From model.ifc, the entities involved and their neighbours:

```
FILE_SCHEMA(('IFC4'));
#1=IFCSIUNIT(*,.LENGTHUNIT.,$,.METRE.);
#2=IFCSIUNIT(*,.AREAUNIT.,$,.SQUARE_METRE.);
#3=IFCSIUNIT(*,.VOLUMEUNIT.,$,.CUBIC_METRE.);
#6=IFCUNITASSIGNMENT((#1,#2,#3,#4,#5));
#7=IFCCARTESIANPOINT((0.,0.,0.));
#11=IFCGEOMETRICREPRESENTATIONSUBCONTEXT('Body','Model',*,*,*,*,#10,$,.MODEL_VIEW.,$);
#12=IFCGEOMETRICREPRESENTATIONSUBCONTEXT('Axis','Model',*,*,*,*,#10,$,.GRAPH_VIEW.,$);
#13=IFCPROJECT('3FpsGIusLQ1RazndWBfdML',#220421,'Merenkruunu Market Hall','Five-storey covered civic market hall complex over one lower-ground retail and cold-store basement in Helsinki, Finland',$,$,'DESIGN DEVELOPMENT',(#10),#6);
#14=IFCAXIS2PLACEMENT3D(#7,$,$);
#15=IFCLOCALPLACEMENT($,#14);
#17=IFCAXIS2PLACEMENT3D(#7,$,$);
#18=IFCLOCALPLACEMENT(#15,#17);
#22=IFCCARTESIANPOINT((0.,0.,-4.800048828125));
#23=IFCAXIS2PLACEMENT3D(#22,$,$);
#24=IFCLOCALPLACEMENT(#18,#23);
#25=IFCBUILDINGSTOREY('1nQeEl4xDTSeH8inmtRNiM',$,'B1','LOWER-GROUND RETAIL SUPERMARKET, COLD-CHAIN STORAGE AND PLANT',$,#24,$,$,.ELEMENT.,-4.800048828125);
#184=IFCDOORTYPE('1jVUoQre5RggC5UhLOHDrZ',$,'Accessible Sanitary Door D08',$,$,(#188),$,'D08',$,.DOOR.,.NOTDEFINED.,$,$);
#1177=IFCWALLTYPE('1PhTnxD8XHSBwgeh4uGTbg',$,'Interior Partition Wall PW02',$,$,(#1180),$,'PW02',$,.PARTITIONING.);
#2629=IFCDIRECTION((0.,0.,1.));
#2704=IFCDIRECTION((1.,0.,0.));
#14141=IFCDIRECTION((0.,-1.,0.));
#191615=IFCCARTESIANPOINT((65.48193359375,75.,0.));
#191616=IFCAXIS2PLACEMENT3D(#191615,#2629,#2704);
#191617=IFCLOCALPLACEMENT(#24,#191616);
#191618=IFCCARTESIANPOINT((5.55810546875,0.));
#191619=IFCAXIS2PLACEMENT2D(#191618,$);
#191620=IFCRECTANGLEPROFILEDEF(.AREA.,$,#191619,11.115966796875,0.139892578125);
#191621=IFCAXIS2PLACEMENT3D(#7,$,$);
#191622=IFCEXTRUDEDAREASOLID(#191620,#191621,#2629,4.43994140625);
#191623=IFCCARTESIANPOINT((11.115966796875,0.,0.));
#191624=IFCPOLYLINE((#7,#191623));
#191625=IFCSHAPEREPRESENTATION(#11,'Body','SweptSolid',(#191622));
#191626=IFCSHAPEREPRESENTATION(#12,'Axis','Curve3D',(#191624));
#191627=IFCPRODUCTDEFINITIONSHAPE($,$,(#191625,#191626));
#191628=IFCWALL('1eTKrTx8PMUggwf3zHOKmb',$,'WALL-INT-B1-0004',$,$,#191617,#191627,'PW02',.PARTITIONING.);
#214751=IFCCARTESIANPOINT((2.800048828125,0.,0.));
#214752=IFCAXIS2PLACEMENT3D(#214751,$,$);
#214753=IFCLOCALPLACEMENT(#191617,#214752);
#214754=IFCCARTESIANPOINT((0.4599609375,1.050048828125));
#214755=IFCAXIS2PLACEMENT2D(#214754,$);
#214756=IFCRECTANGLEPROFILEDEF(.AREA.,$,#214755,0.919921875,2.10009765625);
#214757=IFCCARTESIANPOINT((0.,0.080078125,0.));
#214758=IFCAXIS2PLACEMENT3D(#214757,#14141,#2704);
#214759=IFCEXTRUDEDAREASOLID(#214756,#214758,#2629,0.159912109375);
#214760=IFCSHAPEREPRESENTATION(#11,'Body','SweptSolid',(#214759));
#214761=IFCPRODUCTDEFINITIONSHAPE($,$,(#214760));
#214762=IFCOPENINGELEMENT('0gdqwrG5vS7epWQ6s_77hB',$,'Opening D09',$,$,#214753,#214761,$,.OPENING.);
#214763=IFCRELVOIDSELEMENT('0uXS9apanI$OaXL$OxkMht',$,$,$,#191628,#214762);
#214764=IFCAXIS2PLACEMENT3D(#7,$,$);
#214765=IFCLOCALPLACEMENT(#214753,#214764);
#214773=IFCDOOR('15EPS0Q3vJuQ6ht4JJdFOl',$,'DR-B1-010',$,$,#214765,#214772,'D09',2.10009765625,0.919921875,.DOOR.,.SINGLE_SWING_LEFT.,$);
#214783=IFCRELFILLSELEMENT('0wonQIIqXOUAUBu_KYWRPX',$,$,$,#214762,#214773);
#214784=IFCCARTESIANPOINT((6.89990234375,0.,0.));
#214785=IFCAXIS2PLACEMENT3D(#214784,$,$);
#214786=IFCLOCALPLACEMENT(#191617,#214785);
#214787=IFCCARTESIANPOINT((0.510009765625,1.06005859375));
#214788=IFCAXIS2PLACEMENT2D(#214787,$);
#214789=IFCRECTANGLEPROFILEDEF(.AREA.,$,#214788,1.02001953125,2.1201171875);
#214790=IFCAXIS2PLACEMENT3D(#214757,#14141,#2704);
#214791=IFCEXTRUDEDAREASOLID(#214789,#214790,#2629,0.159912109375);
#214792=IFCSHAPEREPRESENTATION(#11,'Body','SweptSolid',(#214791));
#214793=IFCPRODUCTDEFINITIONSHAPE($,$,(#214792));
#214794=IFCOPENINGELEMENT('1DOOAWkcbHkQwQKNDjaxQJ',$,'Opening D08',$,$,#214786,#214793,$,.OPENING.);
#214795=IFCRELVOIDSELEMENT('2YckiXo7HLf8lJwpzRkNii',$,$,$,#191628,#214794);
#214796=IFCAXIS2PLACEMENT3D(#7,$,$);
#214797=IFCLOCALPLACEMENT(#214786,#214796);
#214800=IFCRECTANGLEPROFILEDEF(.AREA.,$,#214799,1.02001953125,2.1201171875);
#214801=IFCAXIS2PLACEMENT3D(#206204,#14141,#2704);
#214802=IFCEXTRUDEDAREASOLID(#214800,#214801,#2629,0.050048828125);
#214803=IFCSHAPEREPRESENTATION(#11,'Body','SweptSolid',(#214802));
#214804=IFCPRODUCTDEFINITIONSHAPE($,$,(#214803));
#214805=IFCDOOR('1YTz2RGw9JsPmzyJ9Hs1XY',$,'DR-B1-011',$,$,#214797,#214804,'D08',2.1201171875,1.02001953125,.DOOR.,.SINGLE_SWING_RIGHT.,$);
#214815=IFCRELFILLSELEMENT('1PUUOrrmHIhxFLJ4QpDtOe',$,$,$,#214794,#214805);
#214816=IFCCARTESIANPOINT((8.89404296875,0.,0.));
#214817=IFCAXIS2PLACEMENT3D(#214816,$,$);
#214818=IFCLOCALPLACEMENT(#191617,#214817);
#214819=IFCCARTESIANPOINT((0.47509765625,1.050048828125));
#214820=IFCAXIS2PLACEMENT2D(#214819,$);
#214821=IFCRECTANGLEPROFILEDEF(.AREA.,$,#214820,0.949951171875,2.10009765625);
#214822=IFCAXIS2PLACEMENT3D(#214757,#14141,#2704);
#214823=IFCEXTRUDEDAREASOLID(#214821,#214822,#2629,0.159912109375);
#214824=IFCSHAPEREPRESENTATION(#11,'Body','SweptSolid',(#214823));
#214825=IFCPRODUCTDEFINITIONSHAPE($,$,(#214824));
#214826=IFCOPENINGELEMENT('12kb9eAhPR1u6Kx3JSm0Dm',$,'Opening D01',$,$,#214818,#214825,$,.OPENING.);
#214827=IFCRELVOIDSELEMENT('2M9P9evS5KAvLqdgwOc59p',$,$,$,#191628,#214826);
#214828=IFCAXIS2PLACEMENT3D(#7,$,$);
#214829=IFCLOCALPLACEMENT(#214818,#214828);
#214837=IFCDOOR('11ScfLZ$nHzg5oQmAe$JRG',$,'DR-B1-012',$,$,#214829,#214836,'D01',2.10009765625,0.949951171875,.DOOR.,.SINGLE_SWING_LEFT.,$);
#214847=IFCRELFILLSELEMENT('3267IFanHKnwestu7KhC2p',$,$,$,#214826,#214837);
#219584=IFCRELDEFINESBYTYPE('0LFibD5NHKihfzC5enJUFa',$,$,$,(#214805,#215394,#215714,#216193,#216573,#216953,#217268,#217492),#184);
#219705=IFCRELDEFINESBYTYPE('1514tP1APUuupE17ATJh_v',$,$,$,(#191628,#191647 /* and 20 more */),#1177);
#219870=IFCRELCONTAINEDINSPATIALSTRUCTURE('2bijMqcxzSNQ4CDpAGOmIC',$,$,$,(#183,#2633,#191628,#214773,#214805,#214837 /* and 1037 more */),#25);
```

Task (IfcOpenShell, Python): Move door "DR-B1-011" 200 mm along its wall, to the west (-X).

```python
import ifcopenshell
import ifcopenshell.api.geometry
import ifcopenshell.util.placement
import ifcopenshell.util.unit

model = ifcopenshell.open("model.ifc")
unit_scale = ifcopenshell.util.unit.calculate_unit_scale(model)

door = model.by_guid("1YTz2RGw9JsPmzyJ9Hs1XY")
opening = door.FillsVoids[0].RelatingOpeningElement
wall = opening.VoidsElements[0].RelatingBuildingElement

wall_matrix = ifcopenshell.util.placement.get_local_placement(wall.ObjectPlacement)
shift = wall_matrix[:3, 0] * -0.2 / unit_scale
before = ifcopenshell.util.placement.get_local_placement(door.ObjectPlacement)[:3, 3].copy()

# The door is placed relative to its opening, so it follows when the opening moves.
matrix = ifcopenshell.util.placement.get_local_placement(opening.ObjectPlacement)
matrix[:3, 3] += shift
ifcopenshell.api.geometry.edit_object_placement(
    model, product=opening, matrix=matrix, is_si=False, should_transform_children=True
)

after = ifcopenshell.util.placement.get_local_placement(door.ObjectPlacement)[:3, 3]
print("door moved by", (after - before).round(3) + 0.0)

model.write("model_updated.ifc")
```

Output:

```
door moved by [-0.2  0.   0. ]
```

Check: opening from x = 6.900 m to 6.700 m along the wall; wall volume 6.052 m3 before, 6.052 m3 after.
